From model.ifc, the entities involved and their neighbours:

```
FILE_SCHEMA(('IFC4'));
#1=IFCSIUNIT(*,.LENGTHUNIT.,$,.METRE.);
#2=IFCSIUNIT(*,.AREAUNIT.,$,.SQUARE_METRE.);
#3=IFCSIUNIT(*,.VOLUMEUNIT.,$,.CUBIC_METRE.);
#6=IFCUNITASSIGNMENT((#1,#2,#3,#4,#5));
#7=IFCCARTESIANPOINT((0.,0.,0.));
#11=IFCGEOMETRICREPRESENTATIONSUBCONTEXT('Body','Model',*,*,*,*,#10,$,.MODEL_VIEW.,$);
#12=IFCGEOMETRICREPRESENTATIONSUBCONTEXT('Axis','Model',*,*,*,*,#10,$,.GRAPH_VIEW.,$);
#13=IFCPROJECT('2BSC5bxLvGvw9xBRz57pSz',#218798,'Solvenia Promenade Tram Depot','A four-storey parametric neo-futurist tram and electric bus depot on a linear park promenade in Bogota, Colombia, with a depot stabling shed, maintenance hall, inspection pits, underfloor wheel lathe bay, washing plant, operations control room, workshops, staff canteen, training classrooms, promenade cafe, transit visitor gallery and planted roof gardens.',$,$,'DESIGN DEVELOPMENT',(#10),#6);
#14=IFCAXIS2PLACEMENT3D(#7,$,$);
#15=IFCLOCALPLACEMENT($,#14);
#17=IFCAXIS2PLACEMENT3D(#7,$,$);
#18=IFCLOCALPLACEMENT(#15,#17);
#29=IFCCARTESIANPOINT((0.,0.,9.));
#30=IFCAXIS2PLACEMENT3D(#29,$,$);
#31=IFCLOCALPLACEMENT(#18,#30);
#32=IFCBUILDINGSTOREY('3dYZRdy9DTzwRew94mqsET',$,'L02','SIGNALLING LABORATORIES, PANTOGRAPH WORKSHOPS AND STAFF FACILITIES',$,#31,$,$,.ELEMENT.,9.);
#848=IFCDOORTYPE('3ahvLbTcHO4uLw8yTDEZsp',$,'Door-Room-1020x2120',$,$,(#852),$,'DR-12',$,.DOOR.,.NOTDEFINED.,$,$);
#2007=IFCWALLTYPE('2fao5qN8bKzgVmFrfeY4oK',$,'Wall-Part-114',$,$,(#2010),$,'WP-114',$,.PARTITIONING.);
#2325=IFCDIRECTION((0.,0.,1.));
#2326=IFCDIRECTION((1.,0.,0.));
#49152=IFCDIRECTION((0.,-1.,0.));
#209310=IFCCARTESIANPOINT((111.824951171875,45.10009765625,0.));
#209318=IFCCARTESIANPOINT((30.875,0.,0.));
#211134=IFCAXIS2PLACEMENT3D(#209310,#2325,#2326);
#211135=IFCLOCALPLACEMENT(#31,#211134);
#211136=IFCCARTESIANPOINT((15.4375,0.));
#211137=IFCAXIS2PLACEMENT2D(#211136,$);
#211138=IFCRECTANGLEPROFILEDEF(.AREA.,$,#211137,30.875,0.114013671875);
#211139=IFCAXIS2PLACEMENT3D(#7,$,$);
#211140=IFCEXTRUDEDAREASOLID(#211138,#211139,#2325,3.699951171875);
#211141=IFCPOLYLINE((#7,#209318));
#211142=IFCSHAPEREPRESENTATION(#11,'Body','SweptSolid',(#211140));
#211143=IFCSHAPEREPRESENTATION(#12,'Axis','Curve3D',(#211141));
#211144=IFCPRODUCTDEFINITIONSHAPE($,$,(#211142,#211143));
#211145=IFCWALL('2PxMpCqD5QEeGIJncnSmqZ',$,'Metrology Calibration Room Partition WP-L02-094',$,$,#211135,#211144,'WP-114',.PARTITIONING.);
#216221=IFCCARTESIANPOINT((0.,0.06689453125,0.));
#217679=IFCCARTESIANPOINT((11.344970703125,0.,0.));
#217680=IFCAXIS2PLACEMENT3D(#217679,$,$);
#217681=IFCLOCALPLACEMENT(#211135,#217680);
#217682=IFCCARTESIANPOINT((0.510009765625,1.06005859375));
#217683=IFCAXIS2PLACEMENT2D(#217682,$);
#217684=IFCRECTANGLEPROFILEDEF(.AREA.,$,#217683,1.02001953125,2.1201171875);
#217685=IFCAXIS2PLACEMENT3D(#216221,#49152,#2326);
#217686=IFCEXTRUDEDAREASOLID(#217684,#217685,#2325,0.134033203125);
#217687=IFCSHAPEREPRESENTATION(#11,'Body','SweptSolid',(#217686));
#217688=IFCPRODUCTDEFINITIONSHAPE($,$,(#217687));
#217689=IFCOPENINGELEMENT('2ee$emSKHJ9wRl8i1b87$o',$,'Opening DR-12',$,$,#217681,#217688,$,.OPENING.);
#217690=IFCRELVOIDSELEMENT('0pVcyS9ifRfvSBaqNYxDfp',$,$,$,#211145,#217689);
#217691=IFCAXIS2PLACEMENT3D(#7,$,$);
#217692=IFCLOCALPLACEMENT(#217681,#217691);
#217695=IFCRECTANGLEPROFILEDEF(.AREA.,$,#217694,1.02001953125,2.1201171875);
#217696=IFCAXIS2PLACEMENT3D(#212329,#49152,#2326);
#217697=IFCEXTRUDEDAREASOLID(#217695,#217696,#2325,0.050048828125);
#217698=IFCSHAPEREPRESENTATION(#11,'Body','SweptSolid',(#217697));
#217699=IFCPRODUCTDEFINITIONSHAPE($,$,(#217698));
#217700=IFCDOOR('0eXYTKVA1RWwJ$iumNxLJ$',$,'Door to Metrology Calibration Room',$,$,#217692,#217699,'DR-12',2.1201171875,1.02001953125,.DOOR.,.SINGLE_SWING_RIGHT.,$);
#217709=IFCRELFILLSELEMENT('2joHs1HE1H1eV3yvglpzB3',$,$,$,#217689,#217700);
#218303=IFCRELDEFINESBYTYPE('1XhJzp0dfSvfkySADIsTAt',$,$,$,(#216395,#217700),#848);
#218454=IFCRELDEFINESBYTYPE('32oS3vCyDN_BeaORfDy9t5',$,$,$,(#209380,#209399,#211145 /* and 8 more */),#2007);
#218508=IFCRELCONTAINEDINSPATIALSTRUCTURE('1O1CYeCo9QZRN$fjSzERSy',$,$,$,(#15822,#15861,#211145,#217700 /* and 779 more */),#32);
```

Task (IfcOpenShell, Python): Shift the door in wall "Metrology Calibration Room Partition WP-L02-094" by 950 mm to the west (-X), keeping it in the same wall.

```python
import ifcopenshell
import ifcopenshell.api.geometry
import ifcopenshell.util.placement
import ifcopenshell.util.unit

model = ifcopenshell.open("model.ifc")
unit_scale = ifcopenshell.util.unit.calculate_unit_scale(model)

door = model.by_guid("0eXYTKVA1RWwJ$iumNxLJ$")
opening = door.FillsVoids[0].RelatingOpeningElement
wall = opening.VoidsElements[0].RelatingBuildingElement

wall_matrix = ifcopenshell.util.placement.get_local_placement(wall.ObjectPlacement)
shift = wall_matrix[:3, 0] * -0.95 / unit_scale
before = ifcopenshell.util.placement.get_local_placement(door.ObjectPlacement)[:3, 3].copy()

# The door is placed relative to its opening, so it follows when the opening moves.
matrix = ifcopenshell.util.placement.get_local_placement(opening.ObjectPlacement)
matrix[:3, 3] += shift
ifcopenshell.api.geometry.edit_object_placement(
    model, product=opening, matrix=matrix, is_si=False, should_transform_children=True
)

after = ifcopenshell.util.placement.get_local_placement(door.ObjectPlacement)[:3, 3]
print("door moved by", (after - before).round(3) + 0.0)

model.write("model-out.ifc")
```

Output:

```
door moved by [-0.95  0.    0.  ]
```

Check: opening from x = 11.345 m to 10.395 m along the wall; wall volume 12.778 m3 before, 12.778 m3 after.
